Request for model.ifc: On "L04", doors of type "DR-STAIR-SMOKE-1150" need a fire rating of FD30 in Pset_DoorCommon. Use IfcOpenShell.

First a look at what the model holds.

```python
import ifcopenshell
import ifcopenshell.util.element

model = ifcopenshell.open("model.ifc")
print(model.schema)
storey = next(s for s in model.by_type("IfcBuildingStorey") if s.Name == "L04")
doors = [e for e in ifcopenshell.util.element.get_decomposition(storey) if e.is_a("IfcDoor")]
seen = {}
for e in doors:
    element_type = ifcopenshell.util.element.get_type(e)
    key = (element_type.Name if element_type != e and element_type else None, ifcopenshell.util.element.get_pset(e, "Pset_DoorCommon", "FireRating"))
    seen[key] = seen.get(key, 0) + 1
for (name, value), count in sorted(seen.items(), key=str):
    print(count, "x", name, "|", value)
```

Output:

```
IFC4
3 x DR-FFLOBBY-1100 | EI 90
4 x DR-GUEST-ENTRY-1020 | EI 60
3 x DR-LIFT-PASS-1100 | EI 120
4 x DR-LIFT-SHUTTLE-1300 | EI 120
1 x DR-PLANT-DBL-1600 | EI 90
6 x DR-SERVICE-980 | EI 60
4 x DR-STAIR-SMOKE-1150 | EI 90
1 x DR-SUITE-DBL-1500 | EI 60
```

```python
import ifcopenshell
import ifcopenshell.api.pset
import ifcopenshell.util.element

model = ifcopenshell.open("model.ifc")

storey = next(s for s in model.by_type("IfcBuildingStorey") if s.Name == "L04")
doors = [e for e in ifcopenshell.util.element.get_decomposition(storey) if e.is_a("IfcDoor")]

count = 0
for e in doors:
    element_type = ifcopenshell.util.element.get_type(e)
    if element_type in (None, e) or element_type.Name != "DR-STAIR-SMOKE-1150":
        continue
    # add_pset returns the element's existing set when there is one.
    pset = ifcopenshell.api.pset.add_pset(model, product=e, name="Pset_DoorCommon")
    ifcopenshell.api.pset.edit_pset(model, pset=pset, properties={"FireRating": "FD30"})
    count += 1

print(count, "doors updated")

model.write("model_updated.ifc")
```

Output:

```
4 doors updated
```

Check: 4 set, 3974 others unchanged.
